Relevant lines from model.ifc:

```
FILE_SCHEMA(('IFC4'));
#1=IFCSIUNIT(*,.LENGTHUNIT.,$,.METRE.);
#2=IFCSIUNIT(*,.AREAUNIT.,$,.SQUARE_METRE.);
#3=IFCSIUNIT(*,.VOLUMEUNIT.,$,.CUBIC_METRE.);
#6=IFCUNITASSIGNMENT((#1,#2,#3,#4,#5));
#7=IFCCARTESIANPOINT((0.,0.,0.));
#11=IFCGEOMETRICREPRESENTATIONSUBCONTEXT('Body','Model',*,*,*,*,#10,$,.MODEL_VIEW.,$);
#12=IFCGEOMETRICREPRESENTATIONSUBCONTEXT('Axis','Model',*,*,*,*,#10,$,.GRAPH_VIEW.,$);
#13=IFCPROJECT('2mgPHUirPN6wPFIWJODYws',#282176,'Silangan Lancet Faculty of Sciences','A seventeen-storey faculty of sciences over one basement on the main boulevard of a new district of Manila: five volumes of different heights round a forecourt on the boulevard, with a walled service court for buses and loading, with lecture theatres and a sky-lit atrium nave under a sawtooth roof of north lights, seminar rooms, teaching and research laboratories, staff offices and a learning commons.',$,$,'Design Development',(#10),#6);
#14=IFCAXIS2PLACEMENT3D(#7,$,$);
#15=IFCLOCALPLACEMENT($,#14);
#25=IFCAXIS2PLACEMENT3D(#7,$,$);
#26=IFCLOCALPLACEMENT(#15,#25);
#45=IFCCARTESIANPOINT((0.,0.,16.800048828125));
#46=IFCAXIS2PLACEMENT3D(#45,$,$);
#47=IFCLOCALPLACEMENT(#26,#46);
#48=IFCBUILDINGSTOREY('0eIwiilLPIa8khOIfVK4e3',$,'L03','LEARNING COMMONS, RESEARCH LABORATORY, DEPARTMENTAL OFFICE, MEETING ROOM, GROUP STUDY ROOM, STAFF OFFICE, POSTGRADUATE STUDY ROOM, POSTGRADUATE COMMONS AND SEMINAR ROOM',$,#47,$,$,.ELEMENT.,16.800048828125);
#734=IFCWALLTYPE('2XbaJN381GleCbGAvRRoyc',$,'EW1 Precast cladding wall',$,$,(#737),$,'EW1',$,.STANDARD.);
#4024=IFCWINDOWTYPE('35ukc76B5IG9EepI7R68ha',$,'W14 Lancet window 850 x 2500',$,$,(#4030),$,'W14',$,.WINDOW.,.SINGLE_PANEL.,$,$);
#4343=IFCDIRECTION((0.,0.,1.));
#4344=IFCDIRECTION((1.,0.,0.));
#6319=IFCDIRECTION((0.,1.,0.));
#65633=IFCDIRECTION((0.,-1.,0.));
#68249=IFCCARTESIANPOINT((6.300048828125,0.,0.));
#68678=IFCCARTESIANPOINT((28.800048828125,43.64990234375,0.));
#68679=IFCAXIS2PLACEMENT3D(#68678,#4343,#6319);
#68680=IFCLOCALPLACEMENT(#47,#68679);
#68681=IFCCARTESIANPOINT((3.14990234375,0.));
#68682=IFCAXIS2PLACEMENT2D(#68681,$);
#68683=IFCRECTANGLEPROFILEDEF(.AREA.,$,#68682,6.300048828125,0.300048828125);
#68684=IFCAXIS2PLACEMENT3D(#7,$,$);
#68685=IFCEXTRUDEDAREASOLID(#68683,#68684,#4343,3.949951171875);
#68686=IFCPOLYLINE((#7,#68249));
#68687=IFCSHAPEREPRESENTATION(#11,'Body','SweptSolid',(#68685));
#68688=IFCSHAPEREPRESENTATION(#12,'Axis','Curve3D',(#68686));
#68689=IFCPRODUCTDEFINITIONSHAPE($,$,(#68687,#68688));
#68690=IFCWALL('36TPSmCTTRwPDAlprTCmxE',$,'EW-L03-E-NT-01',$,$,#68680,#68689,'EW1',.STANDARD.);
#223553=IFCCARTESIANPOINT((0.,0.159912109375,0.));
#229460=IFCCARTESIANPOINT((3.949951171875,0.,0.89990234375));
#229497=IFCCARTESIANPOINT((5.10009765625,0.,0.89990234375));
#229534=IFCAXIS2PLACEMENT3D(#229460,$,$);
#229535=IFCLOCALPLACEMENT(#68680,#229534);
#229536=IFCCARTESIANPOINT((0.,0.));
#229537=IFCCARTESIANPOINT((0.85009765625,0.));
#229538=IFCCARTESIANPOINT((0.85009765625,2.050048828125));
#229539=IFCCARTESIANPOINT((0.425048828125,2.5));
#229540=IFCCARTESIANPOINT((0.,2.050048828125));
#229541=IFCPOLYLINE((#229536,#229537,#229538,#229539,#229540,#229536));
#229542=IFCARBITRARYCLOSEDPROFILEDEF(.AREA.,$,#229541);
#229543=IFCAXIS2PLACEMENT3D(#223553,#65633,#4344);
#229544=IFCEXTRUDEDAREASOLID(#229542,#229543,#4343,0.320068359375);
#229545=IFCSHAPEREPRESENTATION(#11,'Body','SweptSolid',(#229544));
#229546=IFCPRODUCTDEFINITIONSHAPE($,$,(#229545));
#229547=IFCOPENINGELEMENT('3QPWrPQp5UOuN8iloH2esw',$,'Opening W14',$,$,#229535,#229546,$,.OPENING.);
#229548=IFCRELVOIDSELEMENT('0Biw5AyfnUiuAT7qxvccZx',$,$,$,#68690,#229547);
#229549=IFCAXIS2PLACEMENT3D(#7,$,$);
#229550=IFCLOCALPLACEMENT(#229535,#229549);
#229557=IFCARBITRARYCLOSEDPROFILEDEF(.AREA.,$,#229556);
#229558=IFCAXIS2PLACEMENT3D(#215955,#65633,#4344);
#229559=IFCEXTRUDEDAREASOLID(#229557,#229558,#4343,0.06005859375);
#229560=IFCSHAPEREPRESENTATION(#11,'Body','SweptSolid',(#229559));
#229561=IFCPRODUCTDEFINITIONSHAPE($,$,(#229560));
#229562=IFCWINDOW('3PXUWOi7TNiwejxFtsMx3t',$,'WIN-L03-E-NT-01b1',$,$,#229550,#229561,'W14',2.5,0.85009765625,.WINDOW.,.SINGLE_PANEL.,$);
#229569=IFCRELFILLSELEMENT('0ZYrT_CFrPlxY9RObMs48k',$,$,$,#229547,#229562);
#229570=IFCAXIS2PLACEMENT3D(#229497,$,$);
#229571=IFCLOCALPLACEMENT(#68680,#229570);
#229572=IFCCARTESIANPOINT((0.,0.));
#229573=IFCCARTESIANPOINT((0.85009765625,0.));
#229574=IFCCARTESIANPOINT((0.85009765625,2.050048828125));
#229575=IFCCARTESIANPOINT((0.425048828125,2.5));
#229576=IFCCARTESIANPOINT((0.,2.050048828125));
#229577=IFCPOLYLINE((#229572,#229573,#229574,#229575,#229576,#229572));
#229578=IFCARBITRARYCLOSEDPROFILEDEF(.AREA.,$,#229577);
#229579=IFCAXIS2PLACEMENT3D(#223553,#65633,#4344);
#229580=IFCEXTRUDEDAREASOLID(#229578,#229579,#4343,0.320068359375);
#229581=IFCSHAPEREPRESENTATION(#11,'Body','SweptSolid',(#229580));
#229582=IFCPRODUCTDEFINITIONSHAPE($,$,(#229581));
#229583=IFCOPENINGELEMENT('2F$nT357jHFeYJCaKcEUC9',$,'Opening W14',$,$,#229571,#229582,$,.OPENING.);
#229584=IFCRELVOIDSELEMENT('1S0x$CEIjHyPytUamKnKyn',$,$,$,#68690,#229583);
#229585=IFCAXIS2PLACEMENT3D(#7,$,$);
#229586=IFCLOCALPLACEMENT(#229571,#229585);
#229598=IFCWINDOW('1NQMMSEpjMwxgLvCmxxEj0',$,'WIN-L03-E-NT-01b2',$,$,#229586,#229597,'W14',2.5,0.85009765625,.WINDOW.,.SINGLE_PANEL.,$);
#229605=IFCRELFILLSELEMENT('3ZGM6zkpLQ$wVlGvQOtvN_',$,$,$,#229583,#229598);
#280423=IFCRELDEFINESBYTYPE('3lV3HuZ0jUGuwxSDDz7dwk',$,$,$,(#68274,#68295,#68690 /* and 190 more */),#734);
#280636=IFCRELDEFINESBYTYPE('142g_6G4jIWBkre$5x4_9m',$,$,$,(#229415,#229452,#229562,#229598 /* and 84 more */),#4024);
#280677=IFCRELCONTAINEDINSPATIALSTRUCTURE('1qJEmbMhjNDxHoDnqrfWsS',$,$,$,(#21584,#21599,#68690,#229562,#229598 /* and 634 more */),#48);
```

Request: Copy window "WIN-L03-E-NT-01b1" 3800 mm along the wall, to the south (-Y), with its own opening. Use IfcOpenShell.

```python
import ifcopenshell
import ifcopenshell.api.feature
import ifcopenshell.api.geometry
import ifcopenshell.api.root
import ifcopenshell.geom
import ifcopenshell.util.element
import ifcopenshell.util.placement
import ifcopenshell.util.shape
import ifcopenshell.util.unit

model = ifcopenshell.open("model.ifc")
unit_scale = ifcopenshell.util.unit.calculate_unit_scale(model)
settings = ifcopenshell.geom.settings()


def volume(element):
    """Net volume in cubic metres, openings subtracted."""
    shape = ifcopenshell.geom.create_shape(settings, element)
    return ifcopenshell.util.shape.get_volume(shape.geometry)


window = model.by_guid("3PXUWOi7TNiwejxFtsMx3t")
opening = window.FillsVoids[0].RelatingOpeningElement
wall = opening.VoidsElements[0].RelatingBuildingElement
before = volume(wall)
shift = ifcopenshell.util.placement.get_local_placement(wall.ObjectPlacement)[:3, 0] * -3.8 / unit_scale

# copy_class copies the void relationship, type, container and properties, but no geometry.
new_opening = ifcopenshell.api.root.copy_class(model, product=opening)
new_opening.Representation = ifcopenshell.util.element.copy_deep(
    model, opening.Representation, exclude=["IfcGeometricRepresentationContext", "IfcRepresentationMap"]
)
new_window = ifcopenshell.api.root.copy_class(model, product=window)
new_window.Representation = ifcopenshell.util.element.copy_deep(
    model, window.Representation, exclude=["IfcGeometricRepresentationContext", "IfcRepresentationMap"]
)
new_window.Tag = None
ifcopenshell.api.feature.add_filling(model, opening=new_opening, element=new_window)

for old, new in ((opening, new_opening), (window, new_window)):
    matrix = ifcopenshell.util.placement.get_local_placement(old.ObjectPlacement)
    matrix[:3, 3] += shift
    ifcopenshell.api.geometry.edit_object_placement(model, product=new, matrix=matrix, is_si=False)

after = volume(wall)

print(f"wall volume {before:.3f} -> {after:.3f} m3")

model.write("model_edited.ifc")
```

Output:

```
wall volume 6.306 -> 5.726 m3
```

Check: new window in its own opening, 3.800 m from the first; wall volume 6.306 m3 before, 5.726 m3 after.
